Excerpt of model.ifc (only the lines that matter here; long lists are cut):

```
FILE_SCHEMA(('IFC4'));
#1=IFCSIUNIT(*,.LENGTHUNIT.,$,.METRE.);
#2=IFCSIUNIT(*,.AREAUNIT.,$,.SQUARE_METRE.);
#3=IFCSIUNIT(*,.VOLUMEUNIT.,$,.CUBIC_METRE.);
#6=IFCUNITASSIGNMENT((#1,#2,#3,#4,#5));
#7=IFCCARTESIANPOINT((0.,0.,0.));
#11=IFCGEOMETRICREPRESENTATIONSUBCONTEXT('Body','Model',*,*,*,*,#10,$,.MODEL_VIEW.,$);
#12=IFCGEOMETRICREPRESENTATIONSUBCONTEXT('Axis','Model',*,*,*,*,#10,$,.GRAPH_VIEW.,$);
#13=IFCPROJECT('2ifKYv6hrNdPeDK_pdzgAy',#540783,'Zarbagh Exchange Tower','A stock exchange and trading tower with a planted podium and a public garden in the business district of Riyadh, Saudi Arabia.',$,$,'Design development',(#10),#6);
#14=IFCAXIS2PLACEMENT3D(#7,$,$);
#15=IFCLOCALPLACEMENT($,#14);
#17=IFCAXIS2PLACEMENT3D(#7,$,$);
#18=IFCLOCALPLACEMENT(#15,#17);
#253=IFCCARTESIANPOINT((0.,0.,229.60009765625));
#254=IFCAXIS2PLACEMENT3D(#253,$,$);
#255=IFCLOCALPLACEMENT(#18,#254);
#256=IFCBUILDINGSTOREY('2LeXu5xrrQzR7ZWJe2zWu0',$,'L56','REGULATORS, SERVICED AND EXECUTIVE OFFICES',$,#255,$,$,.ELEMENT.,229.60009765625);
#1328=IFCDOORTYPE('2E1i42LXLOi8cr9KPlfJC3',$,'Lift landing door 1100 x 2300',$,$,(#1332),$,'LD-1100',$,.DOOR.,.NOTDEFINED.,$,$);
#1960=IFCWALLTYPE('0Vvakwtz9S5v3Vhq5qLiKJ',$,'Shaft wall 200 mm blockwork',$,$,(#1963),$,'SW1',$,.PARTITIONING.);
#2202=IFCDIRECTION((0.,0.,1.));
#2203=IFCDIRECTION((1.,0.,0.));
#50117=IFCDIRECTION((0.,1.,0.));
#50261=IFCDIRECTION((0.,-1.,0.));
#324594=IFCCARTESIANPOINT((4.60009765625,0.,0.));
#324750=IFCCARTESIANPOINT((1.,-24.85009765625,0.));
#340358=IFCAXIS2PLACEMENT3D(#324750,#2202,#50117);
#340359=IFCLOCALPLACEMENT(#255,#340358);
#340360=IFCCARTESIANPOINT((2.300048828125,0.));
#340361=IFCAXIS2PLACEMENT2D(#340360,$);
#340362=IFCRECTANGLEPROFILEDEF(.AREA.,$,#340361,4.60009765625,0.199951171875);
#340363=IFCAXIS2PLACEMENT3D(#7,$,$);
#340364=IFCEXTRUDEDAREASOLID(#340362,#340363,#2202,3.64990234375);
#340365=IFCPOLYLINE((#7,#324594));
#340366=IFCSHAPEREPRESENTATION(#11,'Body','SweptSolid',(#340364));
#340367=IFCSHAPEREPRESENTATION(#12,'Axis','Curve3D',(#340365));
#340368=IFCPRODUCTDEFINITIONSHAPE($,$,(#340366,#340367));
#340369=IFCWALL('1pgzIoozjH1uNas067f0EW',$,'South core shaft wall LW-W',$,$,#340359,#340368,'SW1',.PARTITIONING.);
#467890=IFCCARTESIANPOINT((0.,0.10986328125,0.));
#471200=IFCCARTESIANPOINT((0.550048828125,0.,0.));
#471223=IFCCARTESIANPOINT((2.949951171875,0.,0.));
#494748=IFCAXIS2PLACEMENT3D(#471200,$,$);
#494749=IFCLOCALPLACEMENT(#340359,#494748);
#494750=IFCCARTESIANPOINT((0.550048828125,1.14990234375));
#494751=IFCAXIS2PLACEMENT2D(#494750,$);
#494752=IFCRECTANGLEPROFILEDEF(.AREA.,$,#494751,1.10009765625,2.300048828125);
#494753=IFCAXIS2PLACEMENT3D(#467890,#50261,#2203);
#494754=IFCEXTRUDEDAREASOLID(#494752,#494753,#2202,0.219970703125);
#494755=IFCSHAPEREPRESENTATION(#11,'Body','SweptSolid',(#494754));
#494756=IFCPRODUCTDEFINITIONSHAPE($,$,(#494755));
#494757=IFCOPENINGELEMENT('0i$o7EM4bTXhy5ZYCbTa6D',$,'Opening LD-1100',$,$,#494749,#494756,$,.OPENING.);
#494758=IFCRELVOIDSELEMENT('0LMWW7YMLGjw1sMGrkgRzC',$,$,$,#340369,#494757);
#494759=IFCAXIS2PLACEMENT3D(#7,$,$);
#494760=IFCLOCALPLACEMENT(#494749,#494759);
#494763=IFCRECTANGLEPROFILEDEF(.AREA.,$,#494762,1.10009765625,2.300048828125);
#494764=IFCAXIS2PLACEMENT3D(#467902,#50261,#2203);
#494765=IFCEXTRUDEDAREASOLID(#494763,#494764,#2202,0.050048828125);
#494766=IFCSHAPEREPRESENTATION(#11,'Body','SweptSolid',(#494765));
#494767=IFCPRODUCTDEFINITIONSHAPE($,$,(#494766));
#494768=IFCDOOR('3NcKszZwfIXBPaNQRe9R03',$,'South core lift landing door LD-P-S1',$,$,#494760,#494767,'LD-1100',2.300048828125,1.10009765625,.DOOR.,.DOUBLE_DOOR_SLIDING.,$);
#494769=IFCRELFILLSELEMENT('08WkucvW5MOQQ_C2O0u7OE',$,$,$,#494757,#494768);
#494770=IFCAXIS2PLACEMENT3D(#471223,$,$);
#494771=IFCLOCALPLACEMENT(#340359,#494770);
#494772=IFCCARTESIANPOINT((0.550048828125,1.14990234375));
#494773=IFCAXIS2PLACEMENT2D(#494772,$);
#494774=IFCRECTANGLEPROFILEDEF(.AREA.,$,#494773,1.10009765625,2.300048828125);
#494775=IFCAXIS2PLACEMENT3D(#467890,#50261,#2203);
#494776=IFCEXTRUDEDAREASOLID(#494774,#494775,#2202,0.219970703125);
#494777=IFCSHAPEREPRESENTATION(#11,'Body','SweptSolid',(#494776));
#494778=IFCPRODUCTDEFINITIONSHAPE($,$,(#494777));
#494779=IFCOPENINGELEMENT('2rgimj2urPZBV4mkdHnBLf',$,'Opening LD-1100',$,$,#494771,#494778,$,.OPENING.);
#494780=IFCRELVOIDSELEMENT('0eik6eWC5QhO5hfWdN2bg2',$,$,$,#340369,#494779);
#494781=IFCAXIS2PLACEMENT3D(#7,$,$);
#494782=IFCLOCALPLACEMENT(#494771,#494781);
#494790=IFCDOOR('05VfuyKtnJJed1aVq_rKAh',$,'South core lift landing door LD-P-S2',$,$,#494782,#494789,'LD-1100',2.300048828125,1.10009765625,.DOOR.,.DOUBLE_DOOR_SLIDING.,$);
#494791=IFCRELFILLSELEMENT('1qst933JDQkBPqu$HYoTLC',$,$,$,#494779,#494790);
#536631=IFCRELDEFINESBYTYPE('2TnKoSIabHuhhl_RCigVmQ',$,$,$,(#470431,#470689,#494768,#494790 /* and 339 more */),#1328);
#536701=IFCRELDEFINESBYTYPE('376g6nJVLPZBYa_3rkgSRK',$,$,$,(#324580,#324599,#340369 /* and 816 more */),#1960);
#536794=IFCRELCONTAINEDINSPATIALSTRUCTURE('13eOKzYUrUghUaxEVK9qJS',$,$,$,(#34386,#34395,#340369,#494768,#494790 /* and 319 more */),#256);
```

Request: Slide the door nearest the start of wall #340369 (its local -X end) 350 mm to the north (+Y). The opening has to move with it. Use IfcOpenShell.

```python
import ifcopenshell
import ifcopenshell.api.geometry
import ifcopenshell.util.placement
import ifcopenshell.util.unit

model = ifcopenshell.open("model.ifc")
unit_scale = ifcopenshell.util.unit.calculate_unit_scale(model)

door = model.by_guid("3NcKszZwfIXBPaNQRe9R03")
opening = door.FillsVoids[0].RelatingOpeningElement
wall = opening.VoidsElements[0].RelatingBuildingElement

wall_matrix = ifcopenshell.util.placement.get_local_placement(wall.ObjectPlacement)
shift = wall_matrix[:3, 0] * 0.35 / unit_scale
before = ifcopenshell.util.placement.get_local_placement(door.ObjectPlacement)[:3, 3].copy()

# The door is placed relative to its opening, so it follows when the opening moves.
matrix = ifcopenshell.util.placement.get_local_placement(opening.ObjectPlacement)
matrix[:3, 3] += shift
ifcopenshell.api.geometry.edit_object_placement(
    model, product=opening, matrix=matrix, is_si=False, should_transform_children=True
)

after = ifcopenshell.util.placement.get_local_placement(door.ObjectPlacement)[:3, 3]
print("door moved by", (after - before).round(3) + 0.0)

model.write("model_rev.ifc")
```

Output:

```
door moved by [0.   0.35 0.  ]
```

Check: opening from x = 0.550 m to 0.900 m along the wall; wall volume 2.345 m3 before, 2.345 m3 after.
